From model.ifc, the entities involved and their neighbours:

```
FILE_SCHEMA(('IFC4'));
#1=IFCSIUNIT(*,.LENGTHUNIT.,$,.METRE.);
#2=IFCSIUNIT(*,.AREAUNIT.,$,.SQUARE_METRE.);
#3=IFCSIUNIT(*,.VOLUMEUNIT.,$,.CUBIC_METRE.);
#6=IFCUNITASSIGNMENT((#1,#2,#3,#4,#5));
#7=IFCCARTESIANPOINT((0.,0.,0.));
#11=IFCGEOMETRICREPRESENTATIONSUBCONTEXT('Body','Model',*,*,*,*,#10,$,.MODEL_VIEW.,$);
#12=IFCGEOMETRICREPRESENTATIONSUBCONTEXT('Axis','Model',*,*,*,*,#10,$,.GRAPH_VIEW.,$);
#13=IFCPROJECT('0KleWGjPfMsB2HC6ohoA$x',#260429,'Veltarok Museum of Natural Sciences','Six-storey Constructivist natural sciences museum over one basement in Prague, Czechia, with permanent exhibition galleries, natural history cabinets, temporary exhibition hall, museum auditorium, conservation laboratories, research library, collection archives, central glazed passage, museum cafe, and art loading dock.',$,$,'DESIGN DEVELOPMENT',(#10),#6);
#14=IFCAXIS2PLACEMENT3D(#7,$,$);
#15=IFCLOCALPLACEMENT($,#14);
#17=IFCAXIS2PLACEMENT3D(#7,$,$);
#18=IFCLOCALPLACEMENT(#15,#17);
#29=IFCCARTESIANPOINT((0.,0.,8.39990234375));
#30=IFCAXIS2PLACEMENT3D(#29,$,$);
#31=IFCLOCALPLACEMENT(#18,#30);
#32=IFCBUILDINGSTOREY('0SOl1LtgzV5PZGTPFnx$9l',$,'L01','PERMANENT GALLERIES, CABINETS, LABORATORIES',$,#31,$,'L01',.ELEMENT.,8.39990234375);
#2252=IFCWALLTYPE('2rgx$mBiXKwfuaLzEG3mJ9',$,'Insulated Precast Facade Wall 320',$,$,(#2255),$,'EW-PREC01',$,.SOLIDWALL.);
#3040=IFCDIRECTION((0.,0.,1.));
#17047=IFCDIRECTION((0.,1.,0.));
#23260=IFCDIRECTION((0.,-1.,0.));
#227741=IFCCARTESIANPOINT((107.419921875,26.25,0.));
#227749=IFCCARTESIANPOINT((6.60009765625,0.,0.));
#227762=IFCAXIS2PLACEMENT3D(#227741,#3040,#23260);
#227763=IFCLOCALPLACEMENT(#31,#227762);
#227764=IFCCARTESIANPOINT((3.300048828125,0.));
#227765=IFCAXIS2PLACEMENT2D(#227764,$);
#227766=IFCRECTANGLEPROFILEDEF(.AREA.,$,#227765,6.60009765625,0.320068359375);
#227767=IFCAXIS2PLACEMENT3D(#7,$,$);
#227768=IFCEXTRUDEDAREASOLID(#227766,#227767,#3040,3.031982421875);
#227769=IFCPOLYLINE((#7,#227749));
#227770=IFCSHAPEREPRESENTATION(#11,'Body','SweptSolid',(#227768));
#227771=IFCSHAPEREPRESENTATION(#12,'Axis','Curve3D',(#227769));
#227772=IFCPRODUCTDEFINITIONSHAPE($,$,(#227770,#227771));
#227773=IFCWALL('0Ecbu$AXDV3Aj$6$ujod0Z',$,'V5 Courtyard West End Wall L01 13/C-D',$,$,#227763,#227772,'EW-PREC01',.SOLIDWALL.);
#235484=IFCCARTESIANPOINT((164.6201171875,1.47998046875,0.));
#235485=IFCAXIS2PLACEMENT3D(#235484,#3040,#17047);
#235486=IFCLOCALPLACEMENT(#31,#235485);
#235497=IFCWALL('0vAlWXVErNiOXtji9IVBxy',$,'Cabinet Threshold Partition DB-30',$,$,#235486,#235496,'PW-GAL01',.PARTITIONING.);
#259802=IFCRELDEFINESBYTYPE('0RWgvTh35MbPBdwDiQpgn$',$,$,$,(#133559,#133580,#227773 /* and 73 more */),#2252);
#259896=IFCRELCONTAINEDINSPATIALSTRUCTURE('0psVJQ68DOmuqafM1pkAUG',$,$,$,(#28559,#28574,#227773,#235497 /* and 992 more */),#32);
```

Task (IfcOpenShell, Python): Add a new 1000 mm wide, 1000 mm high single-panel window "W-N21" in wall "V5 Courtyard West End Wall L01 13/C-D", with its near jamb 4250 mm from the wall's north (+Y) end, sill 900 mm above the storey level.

```python
import numpy as np
import ifcopenshell
import ifcopenshell.api.feature
import ifcopenshell.api.geometry
import ifcopenshell.api.root
import ifcopenshell.api.spatial
import ifcopenshell.geom
import ifcopenshell.util.element
import ifcopenshell.util.placement
import ifcopenshell.util.representation
import ifcopenshell.util.shape
import ifcopenshell.util.unit

model = ifcopenshell.open("model.ifc")
unit_scale = ifcopenshell.util.unit.calculate_unit_scale(model)
settings = ifcopenshell.geom.settings()


def volume(element):
    """Net volume in cubic metres, openings subtracted."""
    shape = ifcopenshell.geom.create_shape(settings, element)
    return ifcopenshell.util.shape.get_volume(shape.geometry)


wall = model.by_guid("0Ecbu$AXDV3Aj$6$ujod0Z")
storey = ifcopenshell.util.element.get_container(wall, ifc_class="IfcBuildingStorey")
context = ifcopenshell.util.representation.get_context(model, "Model", "Body", "MODEL_VIEW")
before = volume(wall)

width, height, from_end, sill = 1, 1, 4.25, 0.9  # metres

# The wall runs along its own X axis, and the end named is its -X end.
wall_shape = ifcopenshell.geom.create_shape(settings, wall)
x, y, z = ifcopenshell.util.shape.get_vertices(wall_shape.geometry).T
start = x.min() + from_end
face, thickness = float(y.min()), float(y.max() - y.min())
wall_matrix = ifcopenshell.util.placement.get_local_placement(wall.ObjectPlacement)
level = ifcopenshell.util.placement.get_local_placement(storey.ObjectPlacement)[2, 3]


def in_wall(x, y):
    """Placement at x, y metres in the wall's axes, at sill height."""
    matrix = wall_matrix.copy()
    matrix[:, 3] = wall_matrix @ np.array([x / unit_scale, y / unit_scale, 0.0, 1.0])
    matrix[2, 3] = level + sill / unit_scale
    return matrix


# Opening: a box that overshoots both wall faces by 50 mm.
opening = ifcopenshell.api.root.create_entity(model, ifc_class="IfcOpeningElement", predefined_type="OPENING")
box = ifcopenshell.api.geometry.add_wall_representation(
    model, context=context, length=width, height=height, thickness=thickness + 0.1
)
ifcopenshell.api.geometry.assign_representation(model, product=opening, representation=box)
ifcopenshell.api.geometry.edit_object_placement(model, product=opening, matrix=in_wall(start, face - 0.05), is_si=False)
ifcopenshell.api.feature.add_feature(model, feature=opening, element=wall)

window = ifcopenshell.api.root.create_entity(model, ifc_class="IfcWindow", name="W-N21", predefined_type="WINDOW")
window.OverallWidth, window.OverallHeight = width / unit_scale, height / unit_scale
window.PartitioningType = "SINGLE_PANEL"
body = ifcopenshell.api.geometry.add_window_representation(
    model,
    context=context,
    overall_width=window.OverallWidth,
    overall_height=window.OverallHeight,
    partition_type="SINGLE_PANEL",
)
ifcopenshell.api.geometry.assign_representation(model, product=window, representation=body)
ifcopenshell.api.spatial.assign_container(model, products=[window], relating_structure=storey)
ifcopenshell.api.feature.add_filling(model, opening=opening, element=window)

# Centre the window in the wall's thickness.
ifcopenshell.api.geometry.edit_object_placement(model, product=window, matrix=in_wall(start, face), is_si=False)
window_shape = ifcopenshell.geom.create_shape(settings, window)
depth = ifcopenshell.util.shape.get_vertices(window_shape.geometry)[:, 1]
offset = face + thickness / 2 - (depth.min() + depth.max()) / 2
ifcopenshell.api.geometry.edit_object_placement(model, product=window, matrix=in_wall(start, offset), is_si=False)

after = volume(wall)

print(f"wall volume {before:.3f} -> {after:.3f} m3")

model.write("model_updated.ifc")
```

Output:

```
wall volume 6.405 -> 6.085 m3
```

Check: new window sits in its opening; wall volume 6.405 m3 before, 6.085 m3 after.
